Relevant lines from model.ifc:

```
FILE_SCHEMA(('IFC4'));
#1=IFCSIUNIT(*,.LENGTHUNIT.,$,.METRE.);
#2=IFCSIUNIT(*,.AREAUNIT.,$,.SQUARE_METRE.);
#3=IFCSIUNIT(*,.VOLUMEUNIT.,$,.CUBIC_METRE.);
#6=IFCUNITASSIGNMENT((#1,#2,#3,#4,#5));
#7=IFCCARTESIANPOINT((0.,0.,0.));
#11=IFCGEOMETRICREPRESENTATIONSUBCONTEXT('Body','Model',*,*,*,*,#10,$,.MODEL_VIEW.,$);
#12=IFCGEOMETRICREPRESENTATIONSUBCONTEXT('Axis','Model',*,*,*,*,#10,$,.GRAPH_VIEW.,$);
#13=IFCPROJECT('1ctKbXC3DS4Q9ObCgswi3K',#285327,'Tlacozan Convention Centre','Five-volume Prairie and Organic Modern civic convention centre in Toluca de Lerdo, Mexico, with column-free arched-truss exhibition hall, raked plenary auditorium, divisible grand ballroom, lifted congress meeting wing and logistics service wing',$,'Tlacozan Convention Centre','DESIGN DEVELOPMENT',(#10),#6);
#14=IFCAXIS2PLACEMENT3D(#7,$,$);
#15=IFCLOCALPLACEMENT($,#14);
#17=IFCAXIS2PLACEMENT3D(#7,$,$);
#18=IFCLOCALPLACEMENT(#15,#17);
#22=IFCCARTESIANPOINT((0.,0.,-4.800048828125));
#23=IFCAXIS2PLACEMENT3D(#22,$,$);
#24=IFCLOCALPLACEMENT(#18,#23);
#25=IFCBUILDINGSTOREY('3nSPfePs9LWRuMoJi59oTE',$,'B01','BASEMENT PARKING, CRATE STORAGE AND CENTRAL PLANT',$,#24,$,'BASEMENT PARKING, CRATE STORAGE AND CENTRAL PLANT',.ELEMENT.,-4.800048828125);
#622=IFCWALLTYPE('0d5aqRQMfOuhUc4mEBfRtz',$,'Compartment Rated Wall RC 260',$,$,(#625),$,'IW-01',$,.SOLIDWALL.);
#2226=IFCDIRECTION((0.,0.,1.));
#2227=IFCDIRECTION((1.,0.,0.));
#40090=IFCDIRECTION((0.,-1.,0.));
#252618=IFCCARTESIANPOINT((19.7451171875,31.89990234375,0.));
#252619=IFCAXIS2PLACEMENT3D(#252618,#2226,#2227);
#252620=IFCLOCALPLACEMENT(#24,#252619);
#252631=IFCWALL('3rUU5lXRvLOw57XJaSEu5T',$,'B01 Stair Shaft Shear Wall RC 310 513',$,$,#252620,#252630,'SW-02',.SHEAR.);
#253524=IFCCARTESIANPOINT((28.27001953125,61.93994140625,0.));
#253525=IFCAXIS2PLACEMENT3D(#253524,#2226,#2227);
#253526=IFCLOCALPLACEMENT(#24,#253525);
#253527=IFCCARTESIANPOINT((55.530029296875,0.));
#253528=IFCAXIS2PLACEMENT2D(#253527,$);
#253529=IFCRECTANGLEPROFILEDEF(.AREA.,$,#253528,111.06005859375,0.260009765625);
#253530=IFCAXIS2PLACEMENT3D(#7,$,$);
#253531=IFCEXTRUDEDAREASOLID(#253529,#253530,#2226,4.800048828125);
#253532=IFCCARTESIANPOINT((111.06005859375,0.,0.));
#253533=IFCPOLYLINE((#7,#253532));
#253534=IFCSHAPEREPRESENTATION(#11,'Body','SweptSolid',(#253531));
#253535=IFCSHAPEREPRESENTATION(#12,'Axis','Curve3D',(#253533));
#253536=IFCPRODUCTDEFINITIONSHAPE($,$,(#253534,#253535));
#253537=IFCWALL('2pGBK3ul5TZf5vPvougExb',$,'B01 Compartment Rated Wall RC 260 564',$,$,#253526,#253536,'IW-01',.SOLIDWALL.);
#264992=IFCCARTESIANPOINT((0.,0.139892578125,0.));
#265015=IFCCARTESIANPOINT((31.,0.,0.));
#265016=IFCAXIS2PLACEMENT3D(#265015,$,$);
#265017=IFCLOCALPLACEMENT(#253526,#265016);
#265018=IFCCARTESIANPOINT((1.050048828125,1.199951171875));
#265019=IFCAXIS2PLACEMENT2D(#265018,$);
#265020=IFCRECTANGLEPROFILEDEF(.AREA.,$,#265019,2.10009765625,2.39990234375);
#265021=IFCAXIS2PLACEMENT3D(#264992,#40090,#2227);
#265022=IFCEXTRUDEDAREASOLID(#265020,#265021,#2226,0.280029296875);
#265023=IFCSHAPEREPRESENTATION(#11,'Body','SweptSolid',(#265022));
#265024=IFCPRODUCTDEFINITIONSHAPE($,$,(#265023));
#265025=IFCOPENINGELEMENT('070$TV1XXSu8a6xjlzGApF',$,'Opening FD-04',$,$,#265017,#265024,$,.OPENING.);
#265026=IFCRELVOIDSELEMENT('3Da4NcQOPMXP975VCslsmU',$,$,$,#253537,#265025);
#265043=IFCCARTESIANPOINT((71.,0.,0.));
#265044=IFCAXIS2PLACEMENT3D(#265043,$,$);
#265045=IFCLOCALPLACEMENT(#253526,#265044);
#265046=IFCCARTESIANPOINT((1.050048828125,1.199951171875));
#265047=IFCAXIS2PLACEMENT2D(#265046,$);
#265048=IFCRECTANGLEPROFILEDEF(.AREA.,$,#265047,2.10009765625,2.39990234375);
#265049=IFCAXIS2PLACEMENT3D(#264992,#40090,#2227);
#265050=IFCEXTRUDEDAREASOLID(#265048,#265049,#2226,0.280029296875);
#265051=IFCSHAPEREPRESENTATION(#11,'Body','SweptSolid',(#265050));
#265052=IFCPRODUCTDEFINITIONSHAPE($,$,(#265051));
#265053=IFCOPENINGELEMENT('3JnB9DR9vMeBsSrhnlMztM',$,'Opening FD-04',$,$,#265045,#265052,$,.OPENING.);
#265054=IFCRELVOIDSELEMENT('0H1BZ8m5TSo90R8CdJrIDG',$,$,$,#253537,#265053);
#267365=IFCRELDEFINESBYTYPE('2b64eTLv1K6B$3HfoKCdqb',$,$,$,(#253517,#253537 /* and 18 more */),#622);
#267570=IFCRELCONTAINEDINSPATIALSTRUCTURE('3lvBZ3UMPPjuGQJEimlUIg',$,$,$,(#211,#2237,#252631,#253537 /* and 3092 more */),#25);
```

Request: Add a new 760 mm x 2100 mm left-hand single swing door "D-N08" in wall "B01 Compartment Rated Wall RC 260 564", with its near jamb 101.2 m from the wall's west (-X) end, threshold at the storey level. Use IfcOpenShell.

```python
import numpy as np
import ifcopenshell
import ifcopenshell.api.feature
import ifcopenshell.api.geometry
import ifcopenshell.api.root
import ifcopenshell.api.spatial
import ifcopenshell.geom
import ifcopenshell.util.element
import ifcopenshell.util.placement
import ifcopenshell.util.representation
import ifcopenshell.util.shape
import ifcopenshell.util.unit

model = ifcopenshell.open("model.ifc")
unit_scale = ifcopenshell.util.unit.calculate_unit_scale(model)
settings = ifcopenshell.geom.settings()


def volume(element):
    """Net volume in cubic metres, openings subtracted."""
    shape = ifcopenshell.geom.create_shape(settings, element)
    return ifcopenshell.util.shape.get_volume(shape.geometry)


wall = model.by_guid("2pGBK3ul5TZf5vPvougExb")
storey = ifcopenshell.util.element.get_container(wall, ifc_class="IfcBuildingStorey")
context = ifcopenshell.util.representation.get_context(model, "Model", "Body", "MODEL_VIEW")
before = volume(wall)

width, height, from_end, sill = 0.76, 2.1, 101.2, 0.0  # metres

# The wall runs along its own X axis, and the end named is its -X end.
wall_shape = ifcopenshell.geom.create_shape(settings, wall)
x, y, z = ifcopenshell.util.shape.get_vertices(wall_shape.geometry).T
start = x.min() + from_end
face, thickness = float(y.min()), float(y.max() - y.min())
wall_matrix = ifcopenshell.util.placement.get_local_placement(wall.ObjectPlacement)
level = ifcopenshell.util.placement.get_local_placement(storey.ObjectPlacement)[2, 3]


def in_wall(x, y):
    """Placement at x, y metres in the wall's axes, at sill height."""
    matrix = wall_matrix.copy()
    matrix[:, 3] = wall_matrix @ np.array([x / unit_scale, y / unit_scale, 0.0, 1.0])
    matrix[2, 3] = level + sill / unit_scale
    return matrix


# Opening: a box that overshoots both wall faces by 50 mm.
opening = ifcopenshell.api.root.create_entity(model, ifc_class="IfcOpeningElement", predefined_type="OPENING")
box = ifcopenshell.api.geometry.add_wall_representation(
    model, context=context, length=width, height=height, thickness=thickness + 0.1
)
ifcopenshell.api.geometry.assign_representation(model, product=opening, representation=box)
ifcopenshell.api.geometry.edit_object_placement(model, product=opening, matrix=in_wall(start, face - 0.05), is_si=False)
ifcopenshell.api.feature.add_feature(model, feature=opening, element=wall)

door = ifcopenshell.api.root.create_entity(model, ifc_class="IfcDoor", name="D-N08", predefined_type="DOOR")
door.OverallWidth, door.OverallHeight = width / unit_scale, height / unit_scale
door.OperationType = "SINGLE_SWING_LEFT"
body = ifcopenshell.api.geometry.add_door_representation(
    model,
    context=context,
    overall_width=door.OverallWidth,
    overall_height=door.OverallHeight,
    operation_type="SINGLE_SWING_LEFT",
    lining_properties={"LiningDepth": thickness / unit_scale, "ThresholdDepth": thickness / unit_scale},
)
ifcopenshell.api.geometry.assign_representation(model, product=door, representation=body)
ifcopenshell.api.spatial.assign_container(model, products=[door], relating_structure=storey)
ifcopenshell.api.feature.add_filling(model, opening=opening, element=door)

# The lining spans the wall, so the door starts at the wall face.
ifcopenshell.api.geometry.edit_object_placement(model, product=door, matrix=in_wall(start, face), is_si=False)

after = volume(wall)

print(f"wall volume {before:.3f} -> {after:.3f} m3")

model.write("model_updated.ifc")
```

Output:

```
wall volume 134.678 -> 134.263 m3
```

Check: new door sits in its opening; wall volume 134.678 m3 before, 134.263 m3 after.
